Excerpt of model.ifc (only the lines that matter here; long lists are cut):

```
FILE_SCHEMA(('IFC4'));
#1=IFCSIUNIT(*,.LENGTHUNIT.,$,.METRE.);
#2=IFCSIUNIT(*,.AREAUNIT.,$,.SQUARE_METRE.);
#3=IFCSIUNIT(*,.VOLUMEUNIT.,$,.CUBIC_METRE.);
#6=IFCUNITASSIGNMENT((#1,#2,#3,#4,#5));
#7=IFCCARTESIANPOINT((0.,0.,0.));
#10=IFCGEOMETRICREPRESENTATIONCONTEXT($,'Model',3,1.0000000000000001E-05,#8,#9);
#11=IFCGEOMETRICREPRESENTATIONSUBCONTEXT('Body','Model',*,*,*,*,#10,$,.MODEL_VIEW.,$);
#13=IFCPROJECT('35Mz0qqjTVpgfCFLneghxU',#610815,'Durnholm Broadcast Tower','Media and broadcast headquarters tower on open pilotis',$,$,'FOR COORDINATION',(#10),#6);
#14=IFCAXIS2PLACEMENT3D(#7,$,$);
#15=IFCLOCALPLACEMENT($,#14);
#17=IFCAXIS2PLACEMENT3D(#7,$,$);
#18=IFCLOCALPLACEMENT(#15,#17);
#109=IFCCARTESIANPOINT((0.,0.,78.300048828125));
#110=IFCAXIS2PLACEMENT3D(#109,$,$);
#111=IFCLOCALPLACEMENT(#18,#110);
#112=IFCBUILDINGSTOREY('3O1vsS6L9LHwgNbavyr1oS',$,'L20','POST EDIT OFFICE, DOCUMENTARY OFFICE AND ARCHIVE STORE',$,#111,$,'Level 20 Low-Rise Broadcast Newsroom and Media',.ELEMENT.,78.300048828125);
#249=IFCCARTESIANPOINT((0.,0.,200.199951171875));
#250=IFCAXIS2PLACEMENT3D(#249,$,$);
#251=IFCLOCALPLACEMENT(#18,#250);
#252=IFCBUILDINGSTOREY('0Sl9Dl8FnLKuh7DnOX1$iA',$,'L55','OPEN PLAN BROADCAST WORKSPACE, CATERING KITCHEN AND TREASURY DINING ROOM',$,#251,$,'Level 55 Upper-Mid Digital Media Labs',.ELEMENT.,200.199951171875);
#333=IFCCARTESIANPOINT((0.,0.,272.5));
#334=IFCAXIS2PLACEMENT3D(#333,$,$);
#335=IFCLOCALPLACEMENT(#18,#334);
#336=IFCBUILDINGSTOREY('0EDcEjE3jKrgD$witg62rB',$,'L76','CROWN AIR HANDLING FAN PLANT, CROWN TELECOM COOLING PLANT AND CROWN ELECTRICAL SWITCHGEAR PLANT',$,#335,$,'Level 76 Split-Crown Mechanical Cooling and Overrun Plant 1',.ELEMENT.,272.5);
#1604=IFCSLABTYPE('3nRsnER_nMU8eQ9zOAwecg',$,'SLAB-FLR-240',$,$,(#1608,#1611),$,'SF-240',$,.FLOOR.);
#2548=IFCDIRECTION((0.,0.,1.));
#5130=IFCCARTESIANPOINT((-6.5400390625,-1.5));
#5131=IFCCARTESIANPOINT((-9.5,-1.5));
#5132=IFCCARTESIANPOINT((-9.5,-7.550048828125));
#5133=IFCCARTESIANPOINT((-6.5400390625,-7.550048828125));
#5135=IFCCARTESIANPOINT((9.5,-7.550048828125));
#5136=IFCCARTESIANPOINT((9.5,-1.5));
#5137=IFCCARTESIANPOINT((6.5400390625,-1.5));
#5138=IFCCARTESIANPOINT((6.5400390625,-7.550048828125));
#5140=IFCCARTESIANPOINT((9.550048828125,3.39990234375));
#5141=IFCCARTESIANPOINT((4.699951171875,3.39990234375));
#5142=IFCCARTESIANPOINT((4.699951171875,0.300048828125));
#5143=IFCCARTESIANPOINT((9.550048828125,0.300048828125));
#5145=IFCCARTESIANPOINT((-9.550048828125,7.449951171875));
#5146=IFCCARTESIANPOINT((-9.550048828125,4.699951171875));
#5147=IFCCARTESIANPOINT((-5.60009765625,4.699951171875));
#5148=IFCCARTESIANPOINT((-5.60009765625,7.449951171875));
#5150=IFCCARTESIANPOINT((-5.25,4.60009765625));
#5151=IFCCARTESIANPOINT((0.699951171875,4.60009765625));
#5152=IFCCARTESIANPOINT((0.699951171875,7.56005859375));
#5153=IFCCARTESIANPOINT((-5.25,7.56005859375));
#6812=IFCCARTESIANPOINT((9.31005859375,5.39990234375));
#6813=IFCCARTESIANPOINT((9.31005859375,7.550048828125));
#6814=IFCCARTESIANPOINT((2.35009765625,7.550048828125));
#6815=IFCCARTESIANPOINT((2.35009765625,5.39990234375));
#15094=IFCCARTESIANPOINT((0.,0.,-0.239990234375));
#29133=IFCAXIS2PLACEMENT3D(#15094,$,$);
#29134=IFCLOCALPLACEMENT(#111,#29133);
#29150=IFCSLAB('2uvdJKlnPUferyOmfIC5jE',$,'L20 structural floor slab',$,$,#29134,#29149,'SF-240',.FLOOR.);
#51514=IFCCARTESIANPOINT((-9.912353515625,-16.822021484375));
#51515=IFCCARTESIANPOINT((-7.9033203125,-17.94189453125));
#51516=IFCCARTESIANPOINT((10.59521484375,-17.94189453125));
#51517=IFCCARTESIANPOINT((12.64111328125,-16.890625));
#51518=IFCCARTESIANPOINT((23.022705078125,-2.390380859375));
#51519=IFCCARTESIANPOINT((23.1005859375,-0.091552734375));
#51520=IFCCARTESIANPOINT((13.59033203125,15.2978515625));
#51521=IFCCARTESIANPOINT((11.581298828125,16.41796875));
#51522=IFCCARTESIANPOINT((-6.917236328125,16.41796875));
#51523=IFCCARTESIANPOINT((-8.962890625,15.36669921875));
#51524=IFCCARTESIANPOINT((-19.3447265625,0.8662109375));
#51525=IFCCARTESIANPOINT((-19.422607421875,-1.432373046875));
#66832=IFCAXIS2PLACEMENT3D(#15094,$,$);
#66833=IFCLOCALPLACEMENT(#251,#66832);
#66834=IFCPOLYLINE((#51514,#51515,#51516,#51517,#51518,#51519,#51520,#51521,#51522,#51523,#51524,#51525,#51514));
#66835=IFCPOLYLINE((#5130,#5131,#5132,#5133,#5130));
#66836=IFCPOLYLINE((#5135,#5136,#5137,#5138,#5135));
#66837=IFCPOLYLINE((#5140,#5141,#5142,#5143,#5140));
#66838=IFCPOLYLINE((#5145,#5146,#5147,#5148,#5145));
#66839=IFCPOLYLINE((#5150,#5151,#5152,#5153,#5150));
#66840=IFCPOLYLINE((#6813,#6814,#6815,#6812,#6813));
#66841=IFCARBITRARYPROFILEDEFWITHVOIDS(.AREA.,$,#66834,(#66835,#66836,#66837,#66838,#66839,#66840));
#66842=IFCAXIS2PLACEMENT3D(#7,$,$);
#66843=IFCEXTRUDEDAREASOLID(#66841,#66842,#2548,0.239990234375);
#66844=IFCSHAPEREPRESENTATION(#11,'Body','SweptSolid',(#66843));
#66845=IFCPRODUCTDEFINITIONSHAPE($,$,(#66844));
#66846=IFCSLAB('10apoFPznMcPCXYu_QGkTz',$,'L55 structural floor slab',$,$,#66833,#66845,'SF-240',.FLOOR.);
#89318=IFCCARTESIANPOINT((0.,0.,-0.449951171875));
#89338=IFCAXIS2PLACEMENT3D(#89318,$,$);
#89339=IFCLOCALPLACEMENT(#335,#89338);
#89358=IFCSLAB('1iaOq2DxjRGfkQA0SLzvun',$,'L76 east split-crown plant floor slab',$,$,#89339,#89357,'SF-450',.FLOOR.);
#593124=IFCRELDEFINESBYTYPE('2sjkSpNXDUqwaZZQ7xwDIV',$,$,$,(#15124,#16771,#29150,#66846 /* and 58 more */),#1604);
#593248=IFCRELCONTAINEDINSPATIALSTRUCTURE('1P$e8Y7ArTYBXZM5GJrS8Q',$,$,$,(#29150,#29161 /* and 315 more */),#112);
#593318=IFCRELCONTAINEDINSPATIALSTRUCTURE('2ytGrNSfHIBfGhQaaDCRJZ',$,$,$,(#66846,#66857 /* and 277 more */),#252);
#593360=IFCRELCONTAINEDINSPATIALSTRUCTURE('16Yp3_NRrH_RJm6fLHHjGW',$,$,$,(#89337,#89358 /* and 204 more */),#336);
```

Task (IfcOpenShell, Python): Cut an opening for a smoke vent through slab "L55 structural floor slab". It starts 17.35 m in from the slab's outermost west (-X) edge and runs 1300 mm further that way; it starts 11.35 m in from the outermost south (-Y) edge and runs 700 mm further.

```python
import numpy as np
import ifcopenshell
import ifcopenshell.api.feature
import ifcopenshell.api.geometry
import ifcopenshell.api.root
import ifcopenshell.geom
import ifcopenshell.util.placement
import ifcopenshell.util.representation
import ifcopenshell.util.shape
import ifcopenshell.util.unit

model = ifcopenshell.open("model.ifc")
unit_scale = ifcopenshell.util.unit.calculate_unit_scale(model)
settings = ifcopenshell.geom.settings()


def volume(element):
    """Net volume in cubic metres, openings subtracted."""
    shape = ifcopenshell.geom.create_shape(settings, element)
    return ifcopenshell.util.shape.get_volume(shape.geometry)


slab = model.by_id(66846)
before = volume(slab)

# Extent in the slab's own axes, in metres. The edges named are its -X and -Y sides.
slab_shape = ifcopenshell.geom.create_shape(settings, slab)
vertices = ifcopenshell.util.shape.get_vertices(slab_shape.geometry)
x_min, y_min, bottom = vertices.min(axis=0)
top = vertices[:, 2].max()

opening = ifcopenshell.api.root.create_entity(model, ifc_class="IfcOpeningElement", name="Smoke vent opening", predefined_type="OPENING")
context = ifcopenshell.util.representation.get_context(model, "Model", "Body", "MODEL_VIEW")
width, depth = 1.3, 0.7
outline = [(0.0, 0.0), (width, 0.0), (width, depth), (0.0, depth), (0.0, 0.0)]
# Overshoot both faces by 50 mm so the cut is clean.
shape = ifcopenshell.api.geometry.add_slab_representation(
    model, context=context, depth=top - bottom + 0.1, polyline=outline
)
ifcopenshell.api.geometry.assign_representation(model, product=opening, representation=shape)

matrix = ifcopenshell.util.placement.get_local_placement(slab.ObjectPlacement)
matrix[:, 3] = matrix @ np.append(np.array([x_min + 17.35, y_min + 11.35, bottom - 0.05]) / unit_scale, 1.0)
ifcopenshell.api.geometry.edit_object_placement(model, product=opening, matrix=matrix, is_si=False)
ifcopenshell.api.feature.add_feature(model, feature=opening, element=slab)

after = volume(slab)

print(f"slab volume {before:.3f} -> {after:.3f} m3")

model.write("model_rev.ifc")
```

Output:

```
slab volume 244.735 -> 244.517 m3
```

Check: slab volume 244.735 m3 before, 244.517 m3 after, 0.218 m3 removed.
